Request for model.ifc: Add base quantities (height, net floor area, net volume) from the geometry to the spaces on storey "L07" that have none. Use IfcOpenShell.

First a look at what the model holds.

```python
import ifcopenshell
import ifcopenshell.util.element
import ifcopenshell.util.unit

model = ifcopenshell.open("model.ifc")
print(model.schema)
for unit_type in ("LENGTHUNIT", "AREAUNIT", "VOLUMEUNIT"):
    print(unit_type, ifcopenshell.util.unit.calculate_unit_scale(model, unit_type))
storey = next(s for s in model.by_type("IfcBuildingStorey") if s.Name == "L07")
spaces = [e for e in ifcopenshell.util.element.get_decomposition(storey) if e.is_a("IfcSpace")]
for e in sorted(spaces, key=lambda e: e.id()):
    print(e.id(), e.is_a(), e.Name, list(ifcopenshell.util.element.get_psets(e, qtos_only=True)), sep=" | ")
```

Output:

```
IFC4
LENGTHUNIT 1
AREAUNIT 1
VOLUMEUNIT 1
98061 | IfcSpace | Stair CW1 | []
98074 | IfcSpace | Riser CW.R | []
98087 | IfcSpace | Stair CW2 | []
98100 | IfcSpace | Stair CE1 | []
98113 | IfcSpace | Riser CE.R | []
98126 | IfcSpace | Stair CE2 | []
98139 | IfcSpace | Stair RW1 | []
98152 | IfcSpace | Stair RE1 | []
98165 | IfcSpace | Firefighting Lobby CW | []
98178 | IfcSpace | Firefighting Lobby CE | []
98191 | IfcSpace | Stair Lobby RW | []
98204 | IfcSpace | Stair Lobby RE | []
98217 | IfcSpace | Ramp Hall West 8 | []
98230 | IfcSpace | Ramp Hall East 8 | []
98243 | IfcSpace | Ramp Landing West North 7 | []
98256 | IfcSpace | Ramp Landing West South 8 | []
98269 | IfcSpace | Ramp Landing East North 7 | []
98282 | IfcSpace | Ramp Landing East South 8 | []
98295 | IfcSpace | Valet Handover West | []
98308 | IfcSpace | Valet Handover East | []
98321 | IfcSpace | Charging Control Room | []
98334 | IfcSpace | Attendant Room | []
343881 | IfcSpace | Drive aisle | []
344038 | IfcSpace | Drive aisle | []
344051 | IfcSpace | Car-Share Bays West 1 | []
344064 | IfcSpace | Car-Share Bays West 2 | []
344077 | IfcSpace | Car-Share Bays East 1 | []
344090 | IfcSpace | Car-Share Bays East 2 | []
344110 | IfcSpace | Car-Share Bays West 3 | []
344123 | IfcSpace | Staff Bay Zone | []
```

```python
import ifcopenshell
import ifcopenshell.api.pset
import ifcopenshell.geom
import ifcopenshell.util.element
import ifcopenshell.util.shape
import ifcopenshell.util.unit

model = ifcopenshell.open("model.ifc")
unit_scale = ifcopenshell.util.unit.calculate_unit_scale(model)
area_scale = ifcopenshell.util.unit.calculate_unit_scale(model, "AREAUNIT")
volume_scale = ifcopenshell.util.unit.calculate_unit_scale(model, "VOLUMEUNIT")
settings = ifcopenshell.geom.settings()

storey = next(s for s in model.by_type("IfcBuildingStorey") if s.Name == "L07")
spaces = [e for e in ifcopenshell.util.element.get_decomposition(storey) if e.is_a("IfcSpace")]

for e in sorted(spaces, key=lambda e: e.id()):
    if ifcopenshell.util.element.get_psets(e, qtos_only=True, should_inherit=False):
        continue
    # Geometry comes back in metres, in the element's own axes.
    shape = ifcopenshell.geom.create_shape(settings, e)
    values = {
        "Height": ifcopenshell.util.shape.get_z(shape.geometry) / unit_scale,
        "NetFloorArea": ifcopenshell.util.shape.get_footprint_area(shape.geometry) / area_scale,
        "NetVolume": ifcopenshell.util.shape.get_volume(shape.geometry) / volume_scale,
    }
    qto = ifcopenshell.api.pset.add_qto(model, product=e, name="Qto_SpaceBaseQuantities")
    ifcopenshell.api.pset.edit_qto(model, qto=qto, properties=values)
    print(e.id(), {k: round(v, 3) for k, v in values.items()})

model.write("model_updated.ifc")
```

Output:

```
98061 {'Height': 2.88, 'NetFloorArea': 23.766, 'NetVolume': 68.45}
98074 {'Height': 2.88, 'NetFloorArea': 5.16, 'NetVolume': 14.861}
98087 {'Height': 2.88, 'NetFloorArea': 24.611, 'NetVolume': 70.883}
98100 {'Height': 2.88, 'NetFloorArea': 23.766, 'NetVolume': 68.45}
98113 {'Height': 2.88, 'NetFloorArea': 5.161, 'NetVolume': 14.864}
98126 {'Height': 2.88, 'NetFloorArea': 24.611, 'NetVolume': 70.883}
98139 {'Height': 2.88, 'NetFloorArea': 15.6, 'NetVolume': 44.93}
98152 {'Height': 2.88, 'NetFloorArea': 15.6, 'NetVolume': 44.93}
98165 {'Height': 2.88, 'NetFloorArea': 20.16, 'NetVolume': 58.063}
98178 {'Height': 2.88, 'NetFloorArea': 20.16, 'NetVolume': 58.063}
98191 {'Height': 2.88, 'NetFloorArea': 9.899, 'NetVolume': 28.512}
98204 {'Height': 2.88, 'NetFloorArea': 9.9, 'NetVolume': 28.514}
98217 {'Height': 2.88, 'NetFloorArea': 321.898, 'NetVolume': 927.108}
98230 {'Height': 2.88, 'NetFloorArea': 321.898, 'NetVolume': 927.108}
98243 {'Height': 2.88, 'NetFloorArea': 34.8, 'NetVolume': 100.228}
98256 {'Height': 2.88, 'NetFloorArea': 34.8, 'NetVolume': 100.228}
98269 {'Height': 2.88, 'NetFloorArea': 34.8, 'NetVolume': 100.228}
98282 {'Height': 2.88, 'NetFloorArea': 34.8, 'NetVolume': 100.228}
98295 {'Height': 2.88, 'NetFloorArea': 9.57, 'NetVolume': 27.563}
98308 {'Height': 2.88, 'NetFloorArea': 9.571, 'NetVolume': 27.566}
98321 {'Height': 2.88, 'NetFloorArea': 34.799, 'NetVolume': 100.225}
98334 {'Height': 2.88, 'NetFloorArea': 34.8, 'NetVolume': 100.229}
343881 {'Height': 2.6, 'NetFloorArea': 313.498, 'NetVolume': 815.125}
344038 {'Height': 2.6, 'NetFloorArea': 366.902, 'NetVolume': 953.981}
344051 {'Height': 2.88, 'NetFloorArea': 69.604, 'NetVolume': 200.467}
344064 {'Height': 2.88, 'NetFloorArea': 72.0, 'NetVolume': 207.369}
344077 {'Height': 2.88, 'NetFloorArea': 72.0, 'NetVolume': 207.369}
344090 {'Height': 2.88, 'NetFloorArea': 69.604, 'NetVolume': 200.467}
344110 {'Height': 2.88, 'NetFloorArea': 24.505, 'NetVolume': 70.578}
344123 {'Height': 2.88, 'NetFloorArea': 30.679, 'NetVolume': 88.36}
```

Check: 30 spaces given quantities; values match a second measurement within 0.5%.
